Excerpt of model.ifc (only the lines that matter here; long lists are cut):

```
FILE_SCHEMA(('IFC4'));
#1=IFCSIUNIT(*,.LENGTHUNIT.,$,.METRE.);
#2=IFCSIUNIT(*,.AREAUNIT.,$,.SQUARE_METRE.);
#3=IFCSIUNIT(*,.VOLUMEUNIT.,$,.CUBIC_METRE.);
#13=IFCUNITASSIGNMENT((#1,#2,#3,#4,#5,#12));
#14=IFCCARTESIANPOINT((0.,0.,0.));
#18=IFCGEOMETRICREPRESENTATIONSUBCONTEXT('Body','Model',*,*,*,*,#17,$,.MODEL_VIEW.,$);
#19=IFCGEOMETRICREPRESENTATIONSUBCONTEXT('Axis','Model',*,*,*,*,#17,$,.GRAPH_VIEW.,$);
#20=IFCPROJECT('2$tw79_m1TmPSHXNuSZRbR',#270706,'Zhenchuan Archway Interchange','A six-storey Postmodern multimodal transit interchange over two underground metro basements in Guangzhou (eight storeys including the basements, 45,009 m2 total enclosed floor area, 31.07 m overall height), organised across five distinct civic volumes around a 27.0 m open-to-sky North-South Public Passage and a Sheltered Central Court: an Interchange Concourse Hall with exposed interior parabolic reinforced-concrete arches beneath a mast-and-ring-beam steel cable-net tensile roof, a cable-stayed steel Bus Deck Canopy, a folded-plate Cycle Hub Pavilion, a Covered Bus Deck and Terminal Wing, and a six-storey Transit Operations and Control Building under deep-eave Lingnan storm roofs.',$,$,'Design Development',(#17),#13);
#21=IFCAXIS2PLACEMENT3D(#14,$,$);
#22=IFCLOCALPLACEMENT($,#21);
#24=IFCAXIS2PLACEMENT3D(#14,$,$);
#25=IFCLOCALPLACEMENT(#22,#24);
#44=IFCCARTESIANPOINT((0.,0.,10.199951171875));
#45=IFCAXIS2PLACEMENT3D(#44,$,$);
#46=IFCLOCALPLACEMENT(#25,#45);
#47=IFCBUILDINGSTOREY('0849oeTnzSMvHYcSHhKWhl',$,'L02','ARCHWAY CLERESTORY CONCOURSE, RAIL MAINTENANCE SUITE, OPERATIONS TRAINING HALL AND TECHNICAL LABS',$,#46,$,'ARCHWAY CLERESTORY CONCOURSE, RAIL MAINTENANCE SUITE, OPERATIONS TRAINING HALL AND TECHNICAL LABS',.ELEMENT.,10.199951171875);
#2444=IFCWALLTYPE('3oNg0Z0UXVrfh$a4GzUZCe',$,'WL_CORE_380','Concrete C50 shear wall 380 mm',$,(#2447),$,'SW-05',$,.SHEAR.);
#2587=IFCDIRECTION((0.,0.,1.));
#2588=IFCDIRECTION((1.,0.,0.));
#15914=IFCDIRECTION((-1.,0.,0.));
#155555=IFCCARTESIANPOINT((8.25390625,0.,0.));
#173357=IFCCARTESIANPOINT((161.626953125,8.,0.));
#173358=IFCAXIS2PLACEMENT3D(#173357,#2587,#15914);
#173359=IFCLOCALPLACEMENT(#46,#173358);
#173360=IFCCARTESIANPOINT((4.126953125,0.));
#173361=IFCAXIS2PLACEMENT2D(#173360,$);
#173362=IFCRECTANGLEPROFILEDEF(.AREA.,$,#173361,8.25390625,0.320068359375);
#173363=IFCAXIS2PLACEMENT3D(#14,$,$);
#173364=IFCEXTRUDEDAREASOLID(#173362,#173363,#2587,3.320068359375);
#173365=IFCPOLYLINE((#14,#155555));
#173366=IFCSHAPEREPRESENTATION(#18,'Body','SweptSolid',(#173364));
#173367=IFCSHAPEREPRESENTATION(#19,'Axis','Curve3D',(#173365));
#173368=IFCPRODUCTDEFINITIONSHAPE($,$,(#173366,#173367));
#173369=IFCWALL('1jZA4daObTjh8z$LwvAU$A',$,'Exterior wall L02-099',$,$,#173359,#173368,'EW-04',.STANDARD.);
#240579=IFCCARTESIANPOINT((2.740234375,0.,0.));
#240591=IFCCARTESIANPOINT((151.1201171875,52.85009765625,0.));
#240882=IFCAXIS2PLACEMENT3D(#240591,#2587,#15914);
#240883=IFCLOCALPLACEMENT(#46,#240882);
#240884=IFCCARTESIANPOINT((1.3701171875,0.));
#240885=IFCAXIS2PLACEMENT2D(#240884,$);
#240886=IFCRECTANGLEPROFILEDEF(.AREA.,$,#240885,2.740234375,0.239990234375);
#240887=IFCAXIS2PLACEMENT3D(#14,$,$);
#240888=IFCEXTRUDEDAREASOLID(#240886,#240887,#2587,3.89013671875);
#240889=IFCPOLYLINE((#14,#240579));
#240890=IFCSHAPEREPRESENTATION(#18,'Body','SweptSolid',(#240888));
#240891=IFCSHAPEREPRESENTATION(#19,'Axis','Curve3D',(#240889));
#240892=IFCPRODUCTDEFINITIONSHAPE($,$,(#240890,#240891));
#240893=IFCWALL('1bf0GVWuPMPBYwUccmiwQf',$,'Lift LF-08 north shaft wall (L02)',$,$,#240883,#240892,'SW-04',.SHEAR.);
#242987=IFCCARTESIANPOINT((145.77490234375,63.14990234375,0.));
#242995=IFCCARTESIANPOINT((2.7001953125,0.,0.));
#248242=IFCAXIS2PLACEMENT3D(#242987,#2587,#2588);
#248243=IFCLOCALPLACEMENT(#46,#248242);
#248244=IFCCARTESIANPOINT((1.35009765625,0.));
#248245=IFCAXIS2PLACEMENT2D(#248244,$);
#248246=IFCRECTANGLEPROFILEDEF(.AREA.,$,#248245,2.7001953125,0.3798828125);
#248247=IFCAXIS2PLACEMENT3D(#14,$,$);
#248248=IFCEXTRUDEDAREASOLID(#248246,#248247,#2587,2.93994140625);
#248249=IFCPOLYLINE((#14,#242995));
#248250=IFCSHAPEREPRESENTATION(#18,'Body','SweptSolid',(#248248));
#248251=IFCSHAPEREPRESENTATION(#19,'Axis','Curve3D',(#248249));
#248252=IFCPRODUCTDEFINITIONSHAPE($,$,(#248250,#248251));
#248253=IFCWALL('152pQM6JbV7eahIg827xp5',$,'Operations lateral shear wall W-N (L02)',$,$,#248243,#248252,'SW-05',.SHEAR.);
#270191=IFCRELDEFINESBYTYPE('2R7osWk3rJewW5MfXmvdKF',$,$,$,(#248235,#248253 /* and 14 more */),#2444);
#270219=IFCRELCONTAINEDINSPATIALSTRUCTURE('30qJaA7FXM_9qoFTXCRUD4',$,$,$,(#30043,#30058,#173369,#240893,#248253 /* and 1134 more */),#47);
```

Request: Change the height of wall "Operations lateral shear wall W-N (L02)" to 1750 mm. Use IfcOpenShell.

```python
import ifcopenshell
import ifcopenshell.geom
import ifcopenshell.util.representation
import ifcopenshell.util.shape
import ifcopenshell.util.unit

model = ifcopenshell.open("model.ifc")
unit_scale = ifcopenshell.util.unit.calculate_unit_scale(model)
settings = ifcopenshell.geom.settings()


def volume(element):
    """Net volume in cubic metres, openings subtracted."""
    shape = ifcopenshell.geom.create_shape(settings, element)
    return ifcopenshell.util.shape.get_volume(shape.geometry)


wall = model.by_guid("152pQM6JbV7eahIg827xp5")
before = volume(wall)

body = ifcopenshell.util.representation.get_representation(wall, "Model", "Body")
solid = body.Items[0]
old_height = solid.Depth
solid.Depth = 1.75 / unit_scale
after = volume(wall)

print(f"height {old_height:g} -> {solid.Depth:g}, volume {before:.3f} -> {after:.3f} m3")

model.write("model_updated.ifc")
```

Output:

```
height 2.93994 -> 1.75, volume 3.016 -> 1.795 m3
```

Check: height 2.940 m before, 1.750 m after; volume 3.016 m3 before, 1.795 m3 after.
